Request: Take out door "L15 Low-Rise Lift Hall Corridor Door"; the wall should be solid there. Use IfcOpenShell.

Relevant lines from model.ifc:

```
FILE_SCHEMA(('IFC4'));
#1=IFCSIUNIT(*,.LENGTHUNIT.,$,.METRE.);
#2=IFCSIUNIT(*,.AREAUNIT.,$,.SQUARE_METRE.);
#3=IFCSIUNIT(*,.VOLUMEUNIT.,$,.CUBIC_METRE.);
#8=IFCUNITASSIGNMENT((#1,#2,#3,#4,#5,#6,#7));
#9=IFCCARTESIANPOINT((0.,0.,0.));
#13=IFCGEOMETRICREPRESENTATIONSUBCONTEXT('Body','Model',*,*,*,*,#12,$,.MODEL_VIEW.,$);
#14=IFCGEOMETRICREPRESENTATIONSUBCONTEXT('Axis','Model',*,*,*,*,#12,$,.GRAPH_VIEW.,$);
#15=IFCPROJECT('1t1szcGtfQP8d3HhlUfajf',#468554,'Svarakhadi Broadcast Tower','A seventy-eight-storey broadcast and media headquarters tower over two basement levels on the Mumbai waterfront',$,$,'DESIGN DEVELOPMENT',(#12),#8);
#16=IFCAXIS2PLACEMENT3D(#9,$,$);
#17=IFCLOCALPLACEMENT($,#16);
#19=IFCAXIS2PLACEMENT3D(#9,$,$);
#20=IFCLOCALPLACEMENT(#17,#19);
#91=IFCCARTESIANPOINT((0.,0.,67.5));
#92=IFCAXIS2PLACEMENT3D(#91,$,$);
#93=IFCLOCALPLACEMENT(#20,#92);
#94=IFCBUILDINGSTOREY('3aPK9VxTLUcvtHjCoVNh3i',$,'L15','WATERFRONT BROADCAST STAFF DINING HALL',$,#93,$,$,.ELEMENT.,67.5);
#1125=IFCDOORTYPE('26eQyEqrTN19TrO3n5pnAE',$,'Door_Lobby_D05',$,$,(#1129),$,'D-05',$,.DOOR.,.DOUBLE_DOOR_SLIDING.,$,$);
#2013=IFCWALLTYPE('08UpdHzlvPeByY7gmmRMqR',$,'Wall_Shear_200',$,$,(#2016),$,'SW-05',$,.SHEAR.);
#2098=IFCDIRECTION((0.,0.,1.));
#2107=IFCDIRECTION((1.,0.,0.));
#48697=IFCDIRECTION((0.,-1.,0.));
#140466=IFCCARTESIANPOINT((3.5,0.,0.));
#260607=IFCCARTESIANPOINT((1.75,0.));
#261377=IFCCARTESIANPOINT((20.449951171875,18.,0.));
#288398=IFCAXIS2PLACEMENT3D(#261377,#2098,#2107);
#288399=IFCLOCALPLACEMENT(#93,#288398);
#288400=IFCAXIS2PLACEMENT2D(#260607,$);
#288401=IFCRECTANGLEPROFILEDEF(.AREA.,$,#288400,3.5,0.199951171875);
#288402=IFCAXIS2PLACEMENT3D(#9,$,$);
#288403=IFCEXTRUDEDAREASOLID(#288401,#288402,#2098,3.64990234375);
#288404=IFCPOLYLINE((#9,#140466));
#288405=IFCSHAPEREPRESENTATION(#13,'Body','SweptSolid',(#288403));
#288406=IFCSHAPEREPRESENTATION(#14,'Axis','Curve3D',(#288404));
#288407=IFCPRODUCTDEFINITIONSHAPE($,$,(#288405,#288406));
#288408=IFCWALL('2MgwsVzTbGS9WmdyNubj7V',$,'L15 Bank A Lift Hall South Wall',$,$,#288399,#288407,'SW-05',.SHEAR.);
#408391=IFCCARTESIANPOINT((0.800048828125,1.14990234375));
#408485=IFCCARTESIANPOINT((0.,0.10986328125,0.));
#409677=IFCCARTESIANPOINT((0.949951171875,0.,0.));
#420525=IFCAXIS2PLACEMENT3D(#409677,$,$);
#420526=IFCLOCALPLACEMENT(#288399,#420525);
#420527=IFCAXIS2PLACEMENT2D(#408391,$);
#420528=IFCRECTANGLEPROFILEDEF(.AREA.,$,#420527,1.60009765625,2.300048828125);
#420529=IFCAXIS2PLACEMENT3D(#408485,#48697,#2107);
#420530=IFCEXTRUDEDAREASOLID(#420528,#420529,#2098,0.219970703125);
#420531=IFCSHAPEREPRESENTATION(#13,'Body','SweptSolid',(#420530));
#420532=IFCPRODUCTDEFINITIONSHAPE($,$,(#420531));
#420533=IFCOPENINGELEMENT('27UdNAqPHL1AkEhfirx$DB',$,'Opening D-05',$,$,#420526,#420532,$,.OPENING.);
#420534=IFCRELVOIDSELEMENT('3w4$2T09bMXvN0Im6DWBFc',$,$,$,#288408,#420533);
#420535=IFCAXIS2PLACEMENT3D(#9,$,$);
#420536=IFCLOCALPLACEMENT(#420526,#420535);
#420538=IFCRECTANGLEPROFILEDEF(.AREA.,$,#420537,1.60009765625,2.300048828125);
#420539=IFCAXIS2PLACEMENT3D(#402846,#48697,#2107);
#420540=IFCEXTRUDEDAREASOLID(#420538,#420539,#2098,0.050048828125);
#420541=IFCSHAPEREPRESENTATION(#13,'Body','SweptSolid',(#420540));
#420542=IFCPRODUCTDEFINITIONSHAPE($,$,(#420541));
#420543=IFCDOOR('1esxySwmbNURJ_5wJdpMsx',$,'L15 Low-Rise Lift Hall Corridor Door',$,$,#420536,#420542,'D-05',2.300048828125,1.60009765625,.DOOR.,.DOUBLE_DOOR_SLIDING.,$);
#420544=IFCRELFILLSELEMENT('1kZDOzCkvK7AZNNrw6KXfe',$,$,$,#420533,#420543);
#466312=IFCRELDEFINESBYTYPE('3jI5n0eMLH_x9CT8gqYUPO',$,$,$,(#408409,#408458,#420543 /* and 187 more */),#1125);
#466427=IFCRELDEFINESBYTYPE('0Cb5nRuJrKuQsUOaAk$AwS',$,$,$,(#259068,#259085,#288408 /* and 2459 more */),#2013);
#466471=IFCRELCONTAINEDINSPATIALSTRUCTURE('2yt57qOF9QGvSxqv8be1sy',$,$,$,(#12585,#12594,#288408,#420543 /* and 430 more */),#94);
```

```python
import ifcopenshell
import ifcopenshell.api.feature
import ifcopenshell.api.root
import ifcopenshell.geom
import ifcopenshell.util.shape

model = ifcopenshell.open("model.ifc")
settings = ifcopenshell.geom.settings()


def volume(element):
    """Net volume in cubic metres, openings subtracted."""
    shape = ifcopenshell.geom.create_shape(settings, element)
    return ifcopenshell.util.shape.get_volume(shape.geometry)


door = model.by_guid("1esxySwmbNURJ_5wJdpMsx")
opening = door.FillsVoids[0].RelatingOpeningElement
wall = opening.VoidsElements[0].RelatingBuildingElement
before = volume(wall)

ifcopenshell.api.root.remove_product(model, product=door)
ifcopenshell.api.feature.remove_feature(model, feature=opening)

after = volume(wall)

print(f"wall volume {before:.3f} -> {after:.3f} m3")

model.write("model_edited.ifc")
```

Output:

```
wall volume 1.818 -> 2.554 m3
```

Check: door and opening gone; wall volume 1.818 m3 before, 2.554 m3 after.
